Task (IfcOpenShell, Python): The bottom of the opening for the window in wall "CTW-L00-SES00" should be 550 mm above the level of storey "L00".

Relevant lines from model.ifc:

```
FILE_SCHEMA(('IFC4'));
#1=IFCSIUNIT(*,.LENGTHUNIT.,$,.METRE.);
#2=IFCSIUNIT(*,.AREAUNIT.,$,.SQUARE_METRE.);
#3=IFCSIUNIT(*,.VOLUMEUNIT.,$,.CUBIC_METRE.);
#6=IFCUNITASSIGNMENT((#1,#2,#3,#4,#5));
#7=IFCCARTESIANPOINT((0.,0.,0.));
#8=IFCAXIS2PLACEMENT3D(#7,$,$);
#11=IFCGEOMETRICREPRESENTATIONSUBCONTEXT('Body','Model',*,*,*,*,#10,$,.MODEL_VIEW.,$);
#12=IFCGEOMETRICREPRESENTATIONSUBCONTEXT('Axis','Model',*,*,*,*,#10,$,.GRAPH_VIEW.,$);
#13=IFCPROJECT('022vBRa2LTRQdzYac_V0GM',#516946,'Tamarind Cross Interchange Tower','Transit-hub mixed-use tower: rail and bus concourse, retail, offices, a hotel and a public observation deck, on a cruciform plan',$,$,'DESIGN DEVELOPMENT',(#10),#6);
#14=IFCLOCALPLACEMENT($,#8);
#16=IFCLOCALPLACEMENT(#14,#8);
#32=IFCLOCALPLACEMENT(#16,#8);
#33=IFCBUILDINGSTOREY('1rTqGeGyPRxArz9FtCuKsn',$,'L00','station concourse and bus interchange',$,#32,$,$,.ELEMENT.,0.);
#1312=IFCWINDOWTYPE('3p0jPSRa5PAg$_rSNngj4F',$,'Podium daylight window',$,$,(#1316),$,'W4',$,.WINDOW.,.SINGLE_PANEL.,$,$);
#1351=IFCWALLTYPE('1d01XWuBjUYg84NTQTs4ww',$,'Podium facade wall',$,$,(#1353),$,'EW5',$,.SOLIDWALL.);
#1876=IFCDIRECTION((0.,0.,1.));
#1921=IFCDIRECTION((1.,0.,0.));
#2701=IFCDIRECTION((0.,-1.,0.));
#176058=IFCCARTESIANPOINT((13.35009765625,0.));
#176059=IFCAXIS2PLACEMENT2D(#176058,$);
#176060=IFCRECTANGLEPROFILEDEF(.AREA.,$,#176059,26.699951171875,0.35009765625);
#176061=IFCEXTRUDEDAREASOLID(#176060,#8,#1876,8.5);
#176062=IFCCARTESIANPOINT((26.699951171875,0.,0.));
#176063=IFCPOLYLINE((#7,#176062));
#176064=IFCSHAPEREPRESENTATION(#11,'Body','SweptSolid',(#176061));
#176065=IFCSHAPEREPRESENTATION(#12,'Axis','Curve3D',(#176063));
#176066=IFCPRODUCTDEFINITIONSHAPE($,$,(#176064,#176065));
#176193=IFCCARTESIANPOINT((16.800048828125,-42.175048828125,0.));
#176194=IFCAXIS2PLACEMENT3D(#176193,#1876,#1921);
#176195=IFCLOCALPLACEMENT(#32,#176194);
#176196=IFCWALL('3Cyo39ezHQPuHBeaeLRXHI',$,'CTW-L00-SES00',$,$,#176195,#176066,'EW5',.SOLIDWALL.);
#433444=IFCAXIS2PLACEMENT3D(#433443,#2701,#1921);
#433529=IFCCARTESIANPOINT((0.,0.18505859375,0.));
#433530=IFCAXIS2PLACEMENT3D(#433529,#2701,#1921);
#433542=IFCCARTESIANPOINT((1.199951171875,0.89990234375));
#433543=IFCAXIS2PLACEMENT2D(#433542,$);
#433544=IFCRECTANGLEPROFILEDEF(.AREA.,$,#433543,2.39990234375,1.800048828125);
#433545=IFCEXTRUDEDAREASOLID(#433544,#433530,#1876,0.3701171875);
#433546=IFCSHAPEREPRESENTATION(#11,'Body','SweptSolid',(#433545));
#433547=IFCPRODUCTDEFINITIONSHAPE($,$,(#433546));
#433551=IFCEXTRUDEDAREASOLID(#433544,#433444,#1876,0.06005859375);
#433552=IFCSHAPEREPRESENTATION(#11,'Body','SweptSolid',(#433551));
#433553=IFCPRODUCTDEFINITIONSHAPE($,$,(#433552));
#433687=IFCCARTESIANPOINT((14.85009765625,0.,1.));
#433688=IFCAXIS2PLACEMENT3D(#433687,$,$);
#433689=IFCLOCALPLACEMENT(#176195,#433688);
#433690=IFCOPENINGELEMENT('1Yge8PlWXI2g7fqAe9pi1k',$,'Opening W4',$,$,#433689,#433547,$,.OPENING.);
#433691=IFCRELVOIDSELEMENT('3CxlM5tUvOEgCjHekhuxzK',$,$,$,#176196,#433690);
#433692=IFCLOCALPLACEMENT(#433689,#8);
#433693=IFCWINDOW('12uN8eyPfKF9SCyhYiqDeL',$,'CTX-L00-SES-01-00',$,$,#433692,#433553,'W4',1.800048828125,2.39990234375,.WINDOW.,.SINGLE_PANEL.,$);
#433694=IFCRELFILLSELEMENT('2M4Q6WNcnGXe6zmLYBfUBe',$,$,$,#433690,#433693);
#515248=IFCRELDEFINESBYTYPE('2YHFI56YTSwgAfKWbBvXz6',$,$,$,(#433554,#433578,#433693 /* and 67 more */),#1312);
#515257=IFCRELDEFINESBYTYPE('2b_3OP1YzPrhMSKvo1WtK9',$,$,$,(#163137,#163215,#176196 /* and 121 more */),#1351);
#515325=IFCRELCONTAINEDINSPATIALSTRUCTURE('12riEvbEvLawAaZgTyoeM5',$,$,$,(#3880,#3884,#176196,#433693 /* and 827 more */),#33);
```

```python
import numpy as np
import ifcopenshell
import ifcopenshell.api.geometry
import ifcopenshell.geom
import ifcopenshell.util.element
import ifcopenshell.util.placement
import ifcopenshell.util.shape
import ifcopenshell.util.unit

model = ifcopenshell.open("model.ifc")
unit_scale = ifcopenshell.util.unit.calculate_unit_scale(model)

window = model.by_guid("12uN8eyPfKF9SCyhYiqDeL")
opening = window.FillsVoids[0].RelatingOpeningElement
storey = ifcopenshell.util.element.get_container(window, ifc_class="IfcBuildingStorey")
level = ifcopenshell.util.placement.get_local_placement(storey.ObjectPlacement)[2, 3]

# The opening's origin need not be at the sill, so measure its lowest point.
shape = ifcopenshell.geom.create_shape(ifcopenshell.geom.settings(), opening)
bottom = ifcopenshell.util.shape.get_shape_bottom_elevation(shape, shape.geometry) / unit_scale
dz = level + 0.55 / unit_scale - bottom

shift = np.array([0.0, 0.0, dz])
# The window is placed relative to its opening, so it follows when the opening moves.
matrix = ifcopenshell.util.placement.get_local_placement(opening.ObjectPlacement)
matrix[:3, 3] += shift
ifcopenshell.api.geometry.edit_object_placement(
    model, product=opening, matrix=matrix, is_si=False, should_transform_children=True
)

print(f"moved by {dz * unit_scale:+.3f} m")

model.write("model_updated.ifc")
```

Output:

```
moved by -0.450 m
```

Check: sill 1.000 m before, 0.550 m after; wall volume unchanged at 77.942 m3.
